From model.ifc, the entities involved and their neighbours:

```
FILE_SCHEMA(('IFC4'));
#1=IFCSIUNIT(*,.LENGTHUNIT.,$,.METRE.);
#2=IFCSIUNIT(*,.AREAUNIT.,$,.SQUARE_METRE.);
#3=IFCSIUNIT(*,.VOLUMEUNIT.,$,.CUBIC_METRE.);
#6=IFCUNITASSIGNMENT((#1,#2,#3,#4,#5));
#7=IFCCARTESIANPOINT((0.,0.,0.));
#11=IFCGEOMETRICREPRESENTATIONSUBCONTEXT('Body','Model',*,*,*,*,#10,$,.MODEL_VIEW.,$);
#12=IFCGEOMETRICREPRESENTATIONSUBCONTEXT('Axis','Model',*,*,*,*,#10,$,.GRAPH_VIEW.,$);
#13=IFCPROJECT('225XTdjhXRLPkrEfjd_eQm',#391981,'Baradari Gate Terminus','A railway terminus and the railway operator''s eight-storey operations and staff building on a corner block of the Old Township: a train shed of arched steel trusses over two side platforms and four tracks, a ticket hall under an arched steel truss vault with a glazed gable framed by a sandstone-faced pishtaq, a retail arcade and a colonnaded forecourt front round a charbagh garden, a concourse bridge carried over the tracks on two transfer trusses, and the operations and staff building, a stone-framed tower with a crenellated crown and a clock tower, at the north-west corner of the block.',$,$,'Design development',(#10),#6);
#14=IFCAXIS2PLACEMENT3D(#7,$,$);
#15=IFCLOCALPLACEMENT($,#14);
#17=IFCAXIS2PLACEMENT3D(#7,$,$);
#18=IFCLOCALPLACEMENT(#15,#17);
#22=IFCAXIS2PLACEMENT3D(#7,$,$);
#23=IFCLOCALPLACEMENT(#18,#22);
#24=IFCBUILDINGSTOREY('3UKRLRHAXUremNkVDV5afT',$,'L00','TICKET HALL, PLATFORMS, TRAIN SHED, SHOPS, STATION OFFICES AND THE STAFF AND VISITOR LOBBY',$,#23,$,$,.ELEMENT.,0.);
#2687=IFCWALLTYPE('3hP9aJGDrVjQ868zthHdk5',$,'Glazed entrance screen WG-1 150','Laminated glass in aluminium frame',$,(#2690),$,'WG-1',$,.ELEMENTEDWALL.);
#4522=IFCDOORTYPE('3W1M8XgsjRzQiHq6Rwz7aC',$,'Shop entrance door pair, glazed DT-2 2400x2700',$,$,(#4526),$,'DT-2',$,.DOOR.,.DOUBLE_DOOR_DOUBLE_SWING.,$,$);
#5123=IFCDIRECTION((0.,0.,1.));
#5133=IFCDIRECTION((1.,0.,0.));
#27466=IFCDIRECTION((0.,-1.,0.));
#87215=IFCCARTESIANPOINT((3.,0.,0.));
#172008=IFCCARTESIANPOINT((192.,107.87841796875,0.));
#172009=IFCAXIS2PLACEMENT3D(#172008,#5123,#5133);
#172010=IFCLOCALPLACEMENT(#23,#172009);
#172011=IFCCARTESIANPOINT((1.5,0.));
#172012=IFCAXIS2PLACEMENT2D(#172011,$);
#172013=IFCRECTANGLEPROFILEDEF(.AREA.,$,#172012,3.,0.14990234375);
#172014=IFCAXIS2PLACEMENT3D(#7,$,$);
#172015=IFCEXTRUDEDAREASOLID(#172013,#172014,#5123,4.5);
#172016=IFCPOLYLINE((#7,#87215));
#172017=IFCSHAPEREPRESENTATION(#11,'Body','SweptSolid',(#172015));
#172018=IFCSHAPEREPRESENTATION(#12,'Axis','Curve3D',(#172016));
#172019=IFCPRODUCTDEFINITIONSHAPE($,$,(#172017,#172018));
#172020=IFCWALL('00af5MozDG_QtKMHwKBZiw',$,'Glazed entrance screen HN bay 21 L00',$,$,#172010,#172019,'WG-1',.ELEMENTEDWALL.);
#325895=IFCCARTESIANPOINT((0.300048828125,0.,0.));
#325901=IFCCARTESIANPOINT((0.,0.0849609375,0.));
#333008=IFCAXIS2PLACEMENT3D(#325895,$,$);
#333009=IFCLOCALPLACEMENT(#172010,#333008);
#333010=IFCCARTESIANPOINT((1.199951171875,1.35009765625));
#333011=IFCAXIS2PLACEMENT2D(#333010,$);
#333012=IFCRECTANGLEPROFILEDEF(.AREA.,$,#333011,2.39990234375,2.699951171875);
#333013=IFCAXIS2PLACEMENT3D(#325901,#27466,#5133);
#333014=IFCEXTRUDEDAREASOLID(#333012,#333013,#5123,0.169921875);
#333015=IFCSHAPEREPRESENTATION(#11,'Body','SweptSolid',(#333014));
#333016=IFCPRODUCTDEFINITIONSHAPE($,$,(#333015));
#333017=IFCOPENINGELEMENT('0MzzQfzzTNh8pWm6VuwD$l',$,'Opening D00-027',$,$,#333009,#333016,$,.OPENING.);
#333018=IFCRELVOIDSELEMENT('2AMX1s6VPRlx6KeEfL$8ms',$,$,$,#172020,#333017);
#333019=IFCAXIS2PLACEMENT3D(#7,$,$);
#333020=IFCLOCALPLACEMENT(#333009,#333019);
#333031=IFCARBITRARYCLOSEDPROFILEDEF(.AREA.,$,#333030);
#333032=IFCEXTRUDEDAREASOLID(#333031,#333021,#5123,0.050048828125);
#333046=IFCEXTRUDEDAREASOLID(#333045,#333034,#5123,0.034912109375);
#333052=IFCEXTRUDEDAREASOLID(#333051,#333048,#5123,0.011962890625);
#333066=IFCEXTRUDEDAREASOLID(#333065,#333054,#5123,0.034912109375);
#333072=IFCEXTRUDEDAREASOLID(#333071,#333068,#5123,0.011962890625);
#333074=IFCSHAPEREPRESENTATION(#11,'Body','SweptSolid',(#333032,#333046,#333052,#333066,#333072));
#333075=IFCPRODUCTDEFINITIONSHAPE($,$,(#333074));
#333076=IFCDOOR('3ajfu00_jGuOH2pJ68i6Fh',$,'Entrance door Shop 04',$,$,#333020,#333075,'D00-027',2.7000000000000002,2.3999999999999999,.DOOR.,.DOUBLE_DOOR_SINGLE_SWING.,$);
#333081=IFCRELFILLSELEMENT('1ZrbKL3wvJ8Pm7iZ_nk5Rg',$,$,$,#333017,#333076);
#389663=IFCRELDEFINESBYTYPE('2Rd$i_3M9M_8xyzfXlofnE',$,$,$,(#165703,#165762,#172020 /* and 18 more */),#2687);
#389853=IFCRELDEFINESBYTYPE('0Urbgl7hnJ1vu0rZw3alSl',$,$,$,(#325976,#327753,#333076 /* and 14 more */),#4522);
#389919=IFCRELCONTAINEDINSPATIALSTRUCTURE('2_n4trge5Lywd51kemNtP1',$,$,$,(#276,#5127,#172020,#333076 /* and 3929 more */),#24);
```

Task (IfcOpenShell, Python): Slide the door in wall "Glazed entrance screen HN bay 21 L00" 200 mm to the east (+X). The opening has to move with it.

```python
import ifcopenshell
import ifcopenshell.api.geometry
import ifcopenshell.util.placement

model = ifcopenshell.open("model.ifc")

door = model.by_guid("3ajfu00_jGuOH2pJ68i6Fh")
opening = door.FillsVoids[0].RelatingOpeningElement
wall = opening.VoidsElements[0].RelatingBuildingElement

wall_matrix = ifcopenshell.util.placement.get_local_placement(wall.ObjectPlacement)
shift = wall_matrix[:3, 0] * 0.2
before = ifcopenshell.util.placement.get_local_placement(door.ObjectPlacement)[:3, 3].copy()

# The door is placed relative to its opening, so it follows when the opening moves.
matrix = ifcopenshell.util.placement.get_local_placement(opening.ObjectPlacement)
matrix[:3, 3] += shift
ifcopenshell.api.geometry.edit_object_placement(
    model, product=opening, matrix=matrix, is_si=False, should_transform_children=True
)

after = ifcopenshell.util.placement.get_local_placement(door.ObjectPlacement)[:3, 3]
print("door moved by", (after - before).round(3) + 0.0)

model.write("model_updated.ifc")
```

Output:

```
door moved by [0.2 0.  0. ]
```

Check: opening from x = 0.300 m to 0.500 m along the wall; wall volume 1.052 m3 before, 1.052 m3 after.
